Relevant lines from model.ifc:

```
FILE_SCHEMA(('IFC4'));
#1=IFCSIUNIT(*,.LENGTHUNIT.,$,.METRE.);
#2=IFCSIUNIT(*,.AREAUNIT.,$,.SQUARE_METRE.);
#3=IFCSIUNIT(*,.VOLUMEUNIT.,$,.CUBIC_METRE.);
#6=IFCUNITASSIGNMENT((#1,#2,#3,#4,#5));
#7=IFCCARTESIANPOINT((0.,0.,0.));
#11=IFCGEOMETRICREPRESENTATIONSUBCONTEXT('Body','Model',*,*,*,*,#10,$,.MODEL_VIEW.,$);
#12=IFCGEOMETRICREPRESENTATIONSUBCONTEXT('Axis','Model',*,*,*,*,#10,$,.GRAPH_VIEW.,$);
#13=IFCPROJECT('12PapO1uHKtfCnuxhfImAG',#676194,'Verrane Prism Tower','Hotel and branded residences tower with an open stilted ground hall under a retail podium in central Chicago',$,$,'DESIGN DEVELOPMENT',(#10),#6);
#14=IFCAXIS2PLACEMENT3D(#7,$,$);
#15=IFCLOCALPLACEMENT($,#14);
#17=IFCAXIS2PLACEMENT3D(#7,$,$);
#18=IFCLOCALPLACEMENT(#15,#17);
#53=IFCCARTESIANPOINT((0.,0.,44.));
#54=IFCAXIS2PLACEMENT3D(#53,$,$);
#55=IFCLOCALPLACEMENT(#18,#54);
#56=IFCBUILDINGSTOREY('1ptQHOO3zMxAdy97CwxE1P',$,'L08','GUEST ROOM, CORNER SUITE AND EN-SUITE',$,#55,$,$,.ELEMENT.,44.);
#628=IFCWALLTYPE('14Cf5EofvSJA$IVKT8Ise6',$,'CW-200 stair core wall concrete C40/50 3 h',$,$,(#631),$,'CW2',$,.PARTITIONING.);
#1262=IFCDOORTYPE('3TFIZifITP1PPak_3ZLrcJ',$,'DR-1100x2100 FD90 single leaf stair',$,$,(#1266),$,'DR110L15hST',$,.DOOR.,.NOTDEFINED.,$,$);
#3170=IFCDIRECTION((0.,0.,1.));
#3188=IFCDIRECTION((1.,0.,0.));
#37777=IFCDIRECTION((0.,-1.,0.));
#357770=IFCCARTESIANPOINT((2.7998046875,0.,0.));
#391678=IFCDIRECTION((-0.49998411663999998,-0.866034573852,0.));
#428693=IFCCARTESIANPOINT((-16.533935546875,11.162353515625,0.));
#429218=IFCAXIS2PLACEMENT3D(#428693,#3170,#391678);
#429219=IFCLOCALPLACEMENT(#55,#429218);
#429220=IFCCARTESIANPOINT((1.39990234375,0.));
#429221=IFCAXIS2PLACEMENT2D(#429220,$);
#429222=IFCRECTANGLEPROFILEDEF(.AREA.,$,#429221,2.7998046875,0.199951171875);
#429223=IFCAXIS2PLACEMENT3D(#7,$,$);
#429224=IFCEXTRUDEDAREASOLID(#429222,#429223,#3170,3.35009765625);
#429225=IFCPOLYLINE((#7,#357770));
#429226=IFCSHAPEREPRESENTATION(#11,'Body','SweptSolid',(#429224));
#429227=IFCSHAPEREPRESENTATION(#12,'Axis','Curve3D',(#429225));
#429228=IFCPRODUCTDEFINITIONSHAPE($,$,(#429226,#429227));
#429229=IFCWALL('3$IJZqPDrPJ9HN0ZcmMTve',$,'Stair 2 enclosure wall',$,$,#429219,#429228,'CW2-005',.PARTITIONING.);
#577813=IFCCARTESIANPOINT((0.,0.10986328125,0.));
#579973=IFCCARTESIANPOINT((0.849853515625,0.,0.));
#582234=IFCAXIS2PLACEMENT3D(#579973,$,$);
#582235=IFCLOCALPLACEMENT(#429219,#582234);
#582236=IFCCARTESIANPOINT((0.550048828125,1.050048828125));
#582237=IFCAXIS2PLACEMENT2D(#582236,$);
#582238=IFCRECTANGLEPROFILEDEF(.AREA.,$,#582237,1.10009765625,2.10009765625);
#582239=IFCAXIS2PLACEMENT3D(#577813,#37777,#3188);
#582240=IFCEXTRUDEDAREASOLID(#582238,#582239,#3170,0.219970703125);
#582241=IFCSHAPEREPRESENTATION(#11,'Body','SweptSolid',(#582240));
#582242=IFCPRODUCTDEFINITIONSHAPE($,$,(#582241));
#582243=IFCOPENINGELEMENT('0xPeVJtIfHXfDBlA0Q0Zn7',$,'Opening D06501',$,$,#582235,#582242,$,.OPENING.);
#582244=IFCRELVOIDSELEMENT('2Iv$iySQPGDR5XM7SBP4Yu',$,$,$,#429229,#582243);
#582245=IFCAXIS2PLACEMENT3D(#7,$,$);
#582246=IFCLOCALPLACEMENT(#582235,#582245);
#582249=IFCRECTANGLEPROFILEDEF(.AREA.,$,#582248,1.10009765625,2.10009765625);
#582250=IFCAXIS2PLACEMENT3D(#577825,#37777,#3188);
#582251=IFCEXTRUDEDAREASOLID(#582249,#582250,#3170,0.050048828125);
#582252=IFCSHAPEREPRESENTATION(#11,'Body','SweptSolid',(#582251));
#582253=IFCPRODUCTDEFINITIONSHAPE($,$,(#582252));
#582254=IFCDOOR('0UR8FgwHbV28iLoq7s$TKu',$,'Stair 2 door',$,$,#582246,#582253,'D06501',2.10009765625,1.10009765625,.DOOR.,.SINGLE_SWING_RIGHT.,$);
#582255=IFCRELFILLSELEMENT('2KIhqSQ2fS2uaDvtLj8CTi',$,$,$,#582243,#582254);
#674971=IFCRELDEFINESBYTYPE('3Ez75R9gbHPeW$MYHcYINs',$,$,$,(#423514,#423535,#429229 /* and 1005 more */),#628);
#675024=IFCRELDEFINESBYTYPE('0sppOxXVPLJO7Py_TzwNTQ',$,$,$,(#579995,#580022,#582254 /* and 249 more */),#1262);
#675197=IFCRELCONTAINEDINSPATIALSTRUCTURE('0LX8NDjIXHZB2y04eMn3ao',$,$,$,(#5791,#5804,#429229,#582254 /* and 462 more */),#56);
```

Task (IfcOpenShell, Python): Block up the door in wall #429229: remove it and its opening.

```python
import ifcopenshell
import ifcopenshell.api.feature
import ifcopenshell.api.root
import ifcopenshell.geom
import ifcopenshell.util.shape

model = ifcopenshell.open("model.ifc")
settings = ifcopenshell.geom.settings()


def volume(element):
    """Net volume in cubic metres, openings subtracted."""
    shape = ifcopenshell.geom.create_shape(settings, element)
    return ifcopenshell.util.shape.get_volume(shape.geometry)


door = model.by_id(582254)
opening = door.FillsVoids[0].RelatingOpeningElement
wall = opening.VoidsElements[0].RelatingBuildingElement
before = volume(wall)

ifcopenshell.api.root.remove_product(model, product=door)
ifcopenshell.api.feature.remove_feature(model, feature=opening)

after = volume(wall)

print(f"wall volume {before:.3f} -> {after:.3f} m3")

model.write("model_updated.ifc")
```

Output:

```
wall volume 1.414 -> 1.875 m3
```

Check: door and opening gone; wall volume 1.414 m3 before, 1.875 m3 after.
